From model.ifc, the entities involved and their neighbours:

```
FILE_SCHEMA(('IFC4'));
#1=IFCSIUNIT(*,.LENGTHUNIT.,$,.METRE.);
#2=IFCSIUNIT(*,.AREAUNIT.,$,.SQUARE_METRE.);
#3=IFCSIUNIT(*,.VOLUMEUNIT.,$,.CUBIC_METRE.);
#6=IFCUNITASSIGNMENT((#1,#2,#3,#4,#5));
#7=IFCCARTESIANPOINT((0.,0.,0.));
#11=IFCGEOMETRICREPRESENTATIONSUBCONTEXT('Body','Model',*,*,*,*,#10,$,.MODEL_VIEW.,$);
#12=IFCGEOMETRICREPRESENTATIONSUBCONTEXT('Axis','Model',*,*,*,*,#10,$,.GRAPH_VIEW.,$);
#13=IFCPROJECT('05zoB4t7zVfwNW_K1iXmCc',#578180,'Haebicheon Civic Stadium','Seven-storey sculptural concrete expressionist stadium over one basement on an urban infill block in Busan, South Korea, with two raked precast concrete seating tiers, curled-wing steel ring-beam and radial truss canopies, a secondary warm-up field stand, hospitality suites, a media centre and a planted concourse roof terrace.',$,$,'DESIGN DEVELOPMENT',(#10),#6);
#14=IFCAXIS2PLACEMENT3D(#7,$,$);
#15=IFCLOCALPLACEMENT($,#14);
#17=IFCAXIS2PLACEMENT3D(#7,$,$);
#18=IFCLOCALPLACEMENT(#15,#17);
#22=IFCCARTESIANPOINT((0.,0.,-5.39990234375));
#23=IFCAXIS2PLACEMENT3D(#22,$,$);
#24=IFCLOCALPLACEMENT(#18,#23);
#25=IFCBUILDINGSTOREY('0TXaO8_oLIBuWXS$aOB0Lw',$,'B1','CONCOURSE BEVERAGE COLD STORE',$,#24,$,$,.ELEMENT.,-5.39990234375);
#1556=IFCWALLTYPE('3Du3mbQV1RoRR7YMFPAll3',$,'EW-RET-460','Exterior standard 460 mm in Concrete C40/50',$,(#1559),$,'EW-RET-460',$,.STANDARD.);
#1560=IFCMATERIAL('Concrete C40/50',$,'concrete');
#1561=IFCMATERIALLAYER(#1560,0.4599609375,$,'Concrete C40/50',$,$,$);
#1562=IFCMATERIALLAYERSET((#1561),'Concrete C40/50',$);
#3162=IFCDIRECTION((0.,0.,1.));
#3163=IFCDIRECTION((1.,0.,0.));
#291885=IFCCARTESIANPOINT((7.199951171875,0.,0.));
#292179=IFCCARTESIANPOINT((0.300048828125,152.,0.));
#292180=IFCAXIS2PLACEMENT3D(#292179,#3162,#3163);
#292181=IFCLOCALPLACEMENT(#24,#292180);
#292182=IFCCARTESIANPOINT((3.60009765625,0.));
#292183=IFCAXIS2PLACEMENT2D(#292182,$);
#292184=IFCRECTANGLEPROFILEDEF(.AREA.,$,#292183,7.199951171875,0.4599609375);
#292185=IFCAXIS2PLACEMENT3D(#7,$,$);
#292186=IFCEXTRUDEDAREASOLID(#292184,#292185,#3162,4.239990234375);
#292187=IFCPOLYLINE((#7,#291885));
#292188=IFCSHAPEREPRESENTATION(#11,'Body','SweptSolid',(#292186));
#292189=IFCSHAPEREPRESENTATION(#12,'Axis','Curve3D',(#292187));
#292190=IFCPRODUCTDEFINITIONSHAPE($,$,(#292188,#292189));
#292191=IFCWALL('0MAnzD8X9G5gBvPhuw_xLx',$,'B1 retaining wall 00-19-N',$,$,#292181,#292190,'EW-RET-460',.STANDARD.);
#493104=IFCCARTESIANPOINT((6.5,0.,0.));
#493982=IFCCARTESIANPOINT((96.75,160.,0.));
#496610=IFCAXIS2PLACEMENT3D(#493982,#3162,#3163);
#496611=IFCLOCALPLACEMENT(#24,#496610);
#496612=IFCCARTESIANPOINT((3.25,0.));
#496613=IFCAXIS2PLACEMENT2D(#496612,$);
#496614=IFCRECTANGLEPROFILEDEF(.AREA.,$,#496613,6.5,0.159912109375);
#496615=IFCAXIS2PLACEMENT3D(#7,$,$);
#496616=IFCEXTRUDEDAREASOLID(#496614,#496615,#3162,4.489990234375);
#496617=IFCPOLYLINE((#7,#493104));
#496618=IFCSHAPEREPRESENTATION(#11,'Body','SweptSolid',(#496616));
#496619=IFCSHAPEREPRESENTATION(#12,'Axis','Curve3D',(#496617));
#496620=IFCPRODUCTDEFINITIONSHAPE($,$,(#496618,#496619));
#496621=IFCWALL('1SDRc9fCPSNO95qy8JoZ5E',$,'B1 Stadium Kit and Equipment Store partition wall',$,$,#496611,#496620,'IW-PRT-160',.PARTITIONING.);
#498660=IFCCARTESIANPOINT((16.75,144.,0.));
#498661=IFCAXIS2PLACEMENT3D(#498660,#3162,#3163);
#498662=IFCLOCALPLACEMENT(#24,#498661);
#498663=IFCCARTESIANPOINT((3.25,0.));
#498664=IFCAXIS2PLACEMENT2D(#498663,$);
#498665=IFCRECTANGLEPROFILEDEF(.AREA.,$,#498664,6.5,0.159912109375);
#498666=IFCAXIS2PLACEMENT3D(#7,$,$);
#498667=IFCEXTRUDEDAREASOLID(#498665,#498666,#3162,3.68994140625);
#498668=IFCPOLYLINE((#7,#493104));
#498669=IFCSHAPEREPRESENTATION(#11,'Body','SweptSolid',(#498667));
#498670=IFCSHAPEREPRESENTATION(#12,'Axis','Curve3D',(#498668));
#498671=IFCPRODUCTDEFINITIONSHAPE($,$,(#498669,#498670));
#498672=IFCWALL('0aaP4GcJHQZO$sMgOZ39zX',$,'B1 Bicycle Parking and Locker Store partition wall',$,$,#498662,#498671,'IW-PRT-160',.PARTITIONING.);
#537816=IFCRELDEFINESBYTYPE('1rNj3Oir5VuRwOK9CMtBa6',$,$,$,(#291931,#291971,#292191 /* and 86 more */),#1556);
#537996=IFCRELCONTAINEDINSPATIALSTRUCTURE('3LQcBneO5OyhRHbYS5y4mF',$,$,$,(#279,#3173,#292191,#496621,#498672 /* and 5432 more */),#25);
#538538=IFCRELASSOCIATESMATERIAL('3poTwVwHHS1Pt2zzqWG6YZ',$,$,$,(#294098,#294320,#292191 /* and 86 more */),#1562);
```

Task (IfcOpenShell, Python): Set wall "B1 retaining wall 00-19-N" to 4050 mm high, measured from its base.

```python
import ifcopenshell
import ifcopenshell.geom
import ifcopenshell.util.representation
import ifcopenshell.util.shape
import ifcopenshell.util.unit

model = ifcopenshell.open("model.ifc")
unit_scale = ifcopenshell.util.unit.calculate_unit_scale(model)
settings = ifcopenshell.geom.settings()


def volume(element):
    """Net volume in cubic metres, openings subtracted."""
    shape = ifcopenshell.geom.create_shape(settings, element)
    return ifcopenshell.util.shape.get_volume(shape.geometry)


wall = model.by_guid("0MAnzD8X9G5gBvPhuw_xLx")
before = volume(wall)

body = ifcopenshell.util.representation.get_representation(wall, "Model", "Body")
solid = body.Items[0]
old_height = solid.Depth
solid.Depth = 4.05 / unit_scale
after = volume(wall)

print(f"height {old_height:g} -> {solid.Depth:g}, volume {before:.3f} -> {after:.3f} m3")

model.write("model-out.ifc")
```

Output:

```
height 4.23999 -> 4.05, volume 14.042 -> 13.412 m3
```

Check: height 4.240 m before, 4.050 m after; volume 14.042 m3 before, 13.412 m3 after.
